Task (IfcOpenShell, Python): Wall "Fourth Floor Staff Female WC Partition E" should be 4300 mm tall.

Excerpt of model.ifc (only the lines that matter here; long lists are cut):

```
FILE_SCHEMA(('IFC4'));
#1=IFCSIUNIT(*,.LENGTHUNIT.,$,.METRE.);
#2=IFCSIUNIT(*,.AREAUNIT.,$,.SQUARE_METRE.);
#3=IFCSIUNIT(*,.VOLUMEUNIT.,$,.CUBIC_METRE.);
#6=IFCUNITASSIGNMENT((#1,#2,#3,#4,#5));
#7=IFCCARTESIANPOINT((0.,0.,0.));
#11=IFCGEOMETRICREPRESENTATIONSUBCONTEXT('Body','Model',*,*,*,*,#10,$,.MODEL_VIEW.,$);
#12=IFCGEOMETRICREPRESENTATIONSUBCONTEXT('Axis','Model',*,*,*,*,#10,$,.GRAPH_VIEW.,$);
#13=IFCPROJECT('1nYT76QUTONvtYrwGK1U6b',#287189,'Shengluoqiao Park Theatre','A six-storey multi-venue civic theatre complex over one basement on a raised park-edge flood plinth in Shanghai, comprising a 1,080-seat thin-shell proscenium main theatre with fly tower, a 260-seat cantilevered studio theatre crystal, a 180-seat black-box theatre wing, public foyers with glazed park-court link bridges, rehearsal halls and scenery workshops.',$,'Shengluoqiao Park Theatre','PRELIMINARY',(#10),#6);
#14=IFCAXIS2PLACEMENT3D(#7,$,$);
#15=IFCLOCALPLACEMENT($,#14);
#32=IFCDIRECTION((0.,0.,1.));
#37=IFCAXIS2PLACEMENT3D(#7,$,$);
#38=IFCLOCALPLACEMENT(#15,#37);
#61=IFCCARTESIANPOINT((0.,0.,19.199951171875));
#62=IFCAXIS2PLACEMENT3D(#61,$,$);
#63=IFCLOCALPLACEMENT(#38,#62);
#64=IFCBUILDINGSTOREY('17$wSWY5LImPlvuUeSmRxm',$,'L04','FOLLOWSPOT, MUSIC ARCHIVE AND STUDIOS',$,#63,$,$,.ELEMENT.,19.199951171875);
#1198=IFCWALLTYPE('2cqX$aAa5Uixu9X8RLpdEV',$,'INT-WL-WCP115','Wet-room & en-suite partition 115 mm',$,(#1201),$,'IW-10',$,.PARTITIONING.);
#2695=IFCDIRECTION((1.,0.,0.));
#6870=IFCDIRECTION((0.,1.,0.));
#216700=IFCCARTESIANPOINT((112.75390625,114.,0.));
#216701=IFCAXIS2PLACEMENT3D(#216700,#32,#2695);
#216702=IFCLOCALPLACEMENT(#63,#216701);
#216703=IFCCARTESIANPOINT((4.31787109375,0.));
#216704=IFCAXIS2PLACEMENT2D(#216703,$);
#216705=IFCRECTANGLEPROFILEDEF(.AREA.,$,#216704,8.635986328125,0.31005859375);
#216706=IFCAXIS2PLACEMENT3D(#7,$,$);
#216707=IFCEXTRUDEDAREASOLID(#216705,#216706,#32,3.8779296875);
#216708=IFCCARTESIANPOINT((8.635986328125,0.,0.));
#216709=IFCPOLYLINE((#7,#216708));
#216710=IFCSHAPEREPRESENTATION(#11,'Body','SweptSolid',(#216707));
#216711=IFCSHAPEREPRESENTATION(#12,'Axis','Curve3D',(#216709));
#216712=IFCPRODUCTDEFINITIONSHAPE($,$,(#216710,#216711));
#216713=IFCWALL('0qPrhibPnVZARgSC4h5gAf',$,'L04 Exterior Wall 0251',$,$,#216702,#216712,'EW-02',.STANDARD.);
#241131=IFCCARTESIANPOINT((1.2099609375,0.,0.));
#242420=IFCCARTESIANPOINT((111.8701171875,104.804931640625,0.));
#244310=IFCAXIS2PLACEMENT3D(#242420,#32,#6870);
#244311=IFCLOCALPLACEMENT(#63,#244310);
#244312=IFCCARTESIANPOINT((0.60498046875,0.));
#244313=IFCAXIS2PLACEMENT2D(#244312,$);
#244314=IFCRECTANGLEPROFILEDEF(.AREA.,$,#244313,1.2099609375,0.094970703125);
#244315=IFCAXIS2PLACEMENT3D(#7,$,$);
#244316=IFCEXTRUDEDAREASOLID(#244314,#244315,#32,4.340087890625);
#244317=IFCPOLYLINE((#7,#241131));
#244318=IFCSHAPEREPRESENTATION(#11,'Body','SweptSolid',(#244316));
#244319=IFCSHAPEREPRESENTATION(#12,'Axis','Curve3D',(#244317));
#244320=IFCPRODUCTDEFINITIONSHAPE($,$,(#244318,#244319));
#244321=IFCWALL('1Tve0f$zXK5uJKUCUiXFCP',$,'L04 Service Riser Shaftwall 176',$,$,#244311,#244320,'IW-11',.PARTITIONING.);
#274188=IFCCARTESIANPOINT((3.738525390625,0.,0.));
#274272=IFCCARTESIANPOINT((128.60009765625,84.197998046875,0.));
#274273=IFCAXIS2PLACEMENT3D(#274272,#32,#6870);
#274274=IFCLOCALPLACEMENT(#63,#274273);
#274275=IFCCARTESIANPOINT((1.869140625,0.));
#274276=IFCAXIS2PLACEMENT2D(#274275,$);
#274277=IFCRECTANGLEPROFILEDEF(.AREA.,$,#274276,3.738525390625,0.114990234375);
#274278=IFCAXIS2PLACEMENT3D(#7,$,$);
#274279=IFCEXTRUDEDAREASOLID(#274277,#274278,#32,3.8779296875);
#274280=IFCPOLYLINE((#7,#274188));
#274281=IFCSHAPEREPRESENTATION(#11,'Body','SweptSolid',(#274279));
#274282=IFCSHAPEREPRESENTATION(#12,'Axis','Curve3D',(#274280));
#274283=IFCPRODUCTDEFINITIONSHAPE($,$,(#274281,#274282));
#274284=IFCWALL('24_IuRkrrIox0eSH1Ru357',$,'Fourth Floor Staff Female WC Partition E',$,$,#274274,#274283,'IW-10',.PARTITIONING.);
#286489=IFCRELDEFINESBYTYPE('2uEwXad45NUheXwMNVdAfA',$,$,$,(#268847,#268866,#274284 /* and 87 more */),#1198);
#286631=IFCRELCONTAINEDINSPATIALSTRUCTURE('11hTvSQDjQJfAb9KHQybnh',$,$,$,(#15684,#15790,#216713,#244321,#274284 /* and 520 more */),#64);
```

```python
import ifcopenshell
import ifcopenshell.geom
import ifcopenshell.util.representation
import ifcopenshell.util.shape

model = ifcopenshell.open("model.ifc")
settings = ifcopenshell.geom.settings()


def volume(element):
    """Net volume in cubic metres, openings subtracted."""
    shape = ifcopenshell.geom.create_shape(settings, element)
    return ifcopenshell.util.shape.get_volume(shape.geometry)


wall = model.by_guid("24_IuRkrrIox0eSH1Ru357")
before = volume(wall)

body = ifcopenshell.util.representation.get_representation(wall, "Model", "Body")
solid = body.Items[0]
old_height = solid.Depth
solid.Depth = 4.3
after = volume(wall)

print(f"height {old_height:g} -> {solid.Depth:g}, volume {before:.3f} -> {after:.3f} m3")

model.write("model-out.ifc")
```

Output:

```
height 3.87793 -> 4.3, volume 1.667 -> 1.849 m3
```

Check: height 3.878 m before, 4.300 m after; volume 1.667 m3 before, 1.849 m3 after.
